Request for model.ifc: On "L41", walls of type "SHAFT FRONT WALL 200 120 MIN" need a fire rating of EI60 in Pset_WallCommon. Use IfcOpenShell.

First a look at what the model holds.

```python
import ifcopenshell
import ifcopenshell.util.element

model = ifcopenshell.open("model.ifc")
print(model.schema)
storey = next(s for s in model.by_type("IfcBuildingStorey") if s.Name == "L41")
walls = [e for e in ifcopenshell.util.element.get_decomposition(storey) if e.is_a("IfcWall")]
seen = {}
for e in walls:
    element_type = ifcopenshell.util.element.get_type(e)
    key = (element_type.Name if element_type != e and element_type else None, ifcopenshell.util.element.get_pset(e, "Pset_WallCommon", "FireRating"))
    seen[key] = seen.get(key, 0) + 1
for (name, value), count in sorted(seen.items(), key=str):
    print(count, "x", name, "|", value)
```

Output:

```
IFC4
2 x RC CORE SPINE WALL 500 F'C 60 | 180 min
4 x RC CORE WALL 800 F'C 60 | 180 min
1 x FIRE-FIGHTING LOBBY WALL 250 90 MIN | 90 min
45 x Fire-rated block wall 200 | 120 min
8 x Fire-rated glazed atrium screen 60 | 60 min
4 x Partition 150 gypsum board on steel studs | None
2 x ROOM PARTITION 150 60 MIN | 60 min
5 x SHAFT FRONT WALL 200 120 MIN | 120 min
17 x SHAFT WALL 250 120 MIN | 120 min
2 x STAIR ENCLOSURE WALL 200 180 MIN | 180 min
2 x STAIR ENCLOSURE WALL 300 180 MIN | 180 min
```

```python
import ifcopenshell
import ifcopenshell.api.pset
import ifcopenshell.util.element

model = ifcopenshell.open("model.ifc")

storey = next(s for s in model.by_type("IfcBuildingStorey") if s.Name == "L41")
walls = [e for e in ifcopenshell.util.element.get_decomposition(storey) if e.is_a("IfcWall")]

count = 0
for e in walls:
    element_type = ifcopenshell.util.element.get_type(e)
    if element_type in (None, e) or element_type.Name != "SHAFT FRONT WALL 200 120 MIN":
        continue
    found = ifcopenshell.util.element.get_pset(e, "Pset_WallCommon", should_inherit=False)
    if found:
        pset = model.by_id(found["id"])
        if len(ifcopenshell.util.element.get_elements_by_pset(pset)) > 1:
            pset = ifcopenshell.api.pset.unshare_pset(model, products=[e], pset=pset)[0]
    else:
        pset = ifcopenshell.api.pset.add_pset(model, product=e, name="Pset_WallCommon")
    ifcopenshell.api.pset.edit_pset(model, pset=pset, properties={"FireRating": "EI60"})
    count += 1

print(count, "walls updated")

model.write("model_updated.ifc")
```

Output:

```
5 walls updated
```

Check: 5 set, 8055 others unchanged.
